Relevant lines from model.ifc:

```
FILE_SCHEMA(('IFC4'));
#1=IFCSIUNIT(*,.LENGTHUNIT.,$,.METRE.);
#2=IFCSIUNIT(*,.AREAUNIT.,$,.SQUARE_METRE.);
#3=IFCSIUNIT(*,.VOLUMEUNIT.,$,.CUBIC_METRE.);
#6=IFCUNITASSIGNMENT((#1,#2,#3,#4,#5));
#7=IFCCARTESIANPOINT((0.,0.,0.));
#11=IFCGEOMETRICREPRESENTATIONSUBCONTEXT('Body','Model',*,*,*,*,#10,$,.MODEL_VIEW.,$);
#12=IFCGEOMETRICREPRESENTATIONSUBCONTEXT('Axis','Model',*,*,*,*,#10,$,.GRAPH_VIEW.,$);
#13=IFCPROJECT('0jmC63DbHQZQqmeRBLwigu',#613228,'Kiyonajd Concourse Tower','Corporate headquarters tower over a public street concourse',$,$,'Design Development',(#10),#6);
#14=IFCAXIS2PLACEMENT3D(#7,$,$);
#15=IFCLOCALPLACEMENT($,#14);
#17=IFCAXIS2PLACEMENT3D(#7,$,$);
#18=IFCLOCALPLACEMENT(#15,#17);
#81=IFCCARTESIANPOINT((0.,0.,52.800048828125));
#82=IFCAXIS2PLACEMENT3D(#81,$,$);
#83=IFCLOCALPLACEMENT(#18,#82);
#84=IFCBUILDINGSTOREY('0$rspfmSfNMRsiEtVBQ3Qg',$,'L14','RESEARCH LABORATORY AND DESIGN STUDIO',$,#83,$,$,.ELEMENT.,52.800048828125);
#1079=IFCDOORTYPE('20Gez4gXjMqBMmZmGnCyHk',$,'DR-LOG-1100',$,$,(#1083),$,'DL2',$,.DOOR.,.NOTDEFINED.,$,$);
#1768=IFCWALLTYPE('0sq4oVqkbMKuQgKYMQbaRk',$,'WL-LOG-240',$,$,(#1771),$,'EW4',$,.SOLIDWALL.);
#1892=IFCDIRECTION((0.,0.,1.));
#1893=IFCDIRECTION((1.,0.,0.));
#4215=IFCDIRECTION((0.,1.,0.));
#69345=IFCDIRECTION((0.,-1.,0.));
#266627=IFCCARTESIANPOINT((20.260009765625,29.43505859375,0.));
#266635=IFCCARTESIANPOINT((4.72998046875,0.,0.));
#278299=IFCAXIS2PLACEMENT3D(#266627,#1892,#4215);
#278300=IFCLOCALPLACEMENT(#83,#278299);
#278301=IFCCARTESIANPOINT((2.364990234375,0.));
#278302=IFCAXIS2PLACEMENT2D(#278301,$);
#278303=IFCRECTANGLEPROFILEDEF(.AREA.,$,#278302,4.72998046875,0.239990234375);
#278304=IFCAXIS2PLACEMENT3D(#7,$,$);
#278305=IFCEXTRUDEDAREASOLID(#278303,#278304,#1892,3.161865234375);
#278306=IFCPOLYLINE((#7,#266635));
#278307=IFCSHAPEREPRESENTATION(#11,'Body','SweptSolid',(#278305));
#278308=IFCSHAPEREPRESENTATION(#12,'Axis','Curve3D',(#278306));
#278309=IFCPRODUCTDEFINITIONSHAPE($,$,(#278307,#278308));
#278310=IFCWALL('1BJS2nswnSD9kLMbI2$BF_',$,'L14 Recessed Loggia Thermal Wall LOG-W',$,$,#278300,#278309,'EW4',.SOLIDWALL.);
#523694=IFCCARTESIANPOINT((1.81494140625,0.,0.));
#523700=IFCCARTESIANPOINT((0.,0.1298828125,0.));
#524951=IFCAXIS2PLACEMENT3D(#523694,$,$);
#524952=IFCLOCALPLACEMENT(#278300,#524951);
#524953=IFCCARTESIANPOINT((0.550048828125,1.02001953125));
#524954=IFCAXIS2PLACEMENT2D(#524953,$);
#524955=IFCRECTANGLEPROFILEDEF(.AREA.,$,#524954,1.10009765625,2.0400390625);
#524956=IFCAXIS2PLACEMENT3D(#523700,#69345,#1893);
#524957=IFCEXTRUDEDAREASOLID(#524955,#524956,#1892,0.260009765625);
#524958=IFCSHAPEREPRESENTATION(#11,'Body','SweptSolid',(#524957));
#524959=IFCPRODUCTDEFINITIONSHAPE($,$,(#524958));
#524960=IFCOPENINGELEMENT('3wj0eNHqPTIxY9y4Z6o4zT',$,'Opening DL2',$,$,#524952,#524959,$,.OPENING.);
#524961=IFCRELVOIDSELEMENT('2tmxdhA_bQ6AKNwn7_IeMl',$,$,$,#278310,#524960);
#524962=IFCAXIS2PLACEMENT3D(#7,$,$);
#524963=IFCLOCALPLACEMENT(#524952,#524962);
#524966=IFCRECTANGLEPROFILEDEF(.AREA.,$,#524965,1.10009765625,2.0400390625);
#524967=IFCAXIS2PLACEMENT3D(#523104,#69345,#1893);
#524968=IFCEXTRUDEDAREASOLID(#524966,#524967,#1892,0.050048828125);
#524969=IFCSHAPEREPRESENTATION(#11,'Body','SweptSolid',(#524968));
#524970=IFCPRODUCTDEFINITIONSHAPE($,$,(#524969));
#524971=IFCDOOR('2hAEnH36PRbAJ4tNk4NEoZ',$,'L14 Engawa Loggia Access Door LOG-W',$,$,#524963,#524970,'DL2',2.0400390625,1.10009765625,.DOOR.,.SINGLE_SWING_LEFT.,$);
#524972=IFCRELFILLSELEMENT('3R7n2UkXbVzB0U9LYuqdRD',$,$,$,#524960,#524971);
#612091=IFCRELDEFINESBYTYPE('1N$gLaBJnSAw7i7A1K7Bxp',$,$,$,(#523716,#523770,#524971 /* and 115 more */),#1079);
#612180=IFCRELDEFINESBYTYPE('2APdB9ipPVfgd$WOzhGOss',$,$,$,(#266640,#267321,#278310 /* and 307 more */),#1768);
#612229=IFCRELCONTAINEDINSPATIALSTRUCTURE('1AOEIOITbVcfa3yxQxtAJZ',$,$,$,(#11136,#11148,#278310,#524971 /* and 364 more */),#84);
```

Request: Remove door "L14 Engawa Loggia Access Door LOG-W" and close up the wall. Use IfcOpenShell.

```python
import ifcopenshell
import ifcopenshell.api.feature
import ifcopenshell.api.root
import ifcopenshell.geom
import ifcopenshell.util.shape

model = ifcopenshell.open("model.ifc")
settings = ifcopenshell.geom.settings()


def volume(element):
    """Net volume in cubic metres, openings subtracted."""
    shape = ifcopenshell.geom.create_shape(settings, element)
    return ifcopenshell.util.shape.get_volume(shape.geometry)


door = model.by_id(524971)
opening = door.FillsVoids[0].RelatingOpeningElement
wall = opening.VoidsElements[0].RelatingBuildingElement
before = volume(wall)

ifcopenshell.api.root.remove_product(model, product=door)
ifcopenshell.api.feature.remove_feature(model, feature=opening)

after = volume(wall)

print(f"wall volume {before:.3f} -> {after:.3f} m3")

model.write("model_rev.ifc")
```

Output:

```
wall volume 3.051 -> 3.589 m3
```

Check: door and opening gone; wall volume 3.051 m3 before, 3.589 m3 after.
